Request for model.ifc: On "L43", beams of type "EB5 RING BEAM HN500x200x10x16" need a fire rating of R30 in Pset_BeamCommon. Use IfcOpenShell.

First a look at what the model holds.

```python
import ifcopenshell
import ifcopenshell.util.element

model = ifcopenshell.open("model.ifc")
print(model.schema)
storey = next(s for s in model.by_type("IfcBuildingStorey") if s.Name == "L43")
beams = [e for e in ifcopenshell.util.element.get_decomposition(storey) if e.is_a("IfcBeam")]
seen = {}
for e in beams:
    element_type = ifcopenshell.util.element.get_type(e)
    key = (element_type.Name if element_type != e and element_type else None, ifcopenshell.util.element.get_pset(e, "Pset_BeamCommon", "FireRating"))
    seen[key] = seen.get(key, 0) + 1
for (name, value), count in sorted(seen.items(), key=str):
    print(count, "x", name, "|", value)
```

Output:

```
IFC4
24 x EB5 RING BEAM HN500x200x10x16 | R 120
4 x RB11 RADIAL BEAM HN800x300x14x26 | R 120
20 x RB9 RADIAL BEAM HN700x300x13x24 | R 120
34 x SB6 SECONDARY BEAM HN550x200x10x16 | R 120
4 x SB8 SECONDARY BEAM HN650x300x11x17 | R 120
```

```python
import ifcopenshell
import ifcopenshell.api.pset
import ifcopenshell.util.element

model = ifcopenshell.open("model.ifc")

storey = next(s for s in model.by_type("IfcBuildingStorey") if s.Name == "L43")
beams = [e for e in ifcopenshell.util.element.get_decomposition(storey) if e.is_a("IfcBeam")]

count = 0
for e in beams:
    element_type = ifcopenshell.util.element.get_type(e)
    if element_type in (None, e) or element_type.Name != "EB5 RING BEAM HN500x200x10x16":
        continue
    found = ifcopenshell.util.element.get_pset(e, "Pset_BeamCommon", should_inherit=False)
    if found:
        pset = model.by_id(found["id"])
        if len(ifcopenshell.util.element.get_elements_by_pset(pset)) > 1:
            pset = ifcopenshell.api.pset.unshare_pset(model, products=[e], pset=pset)[0]
    else:
        pset = ifcopenshell.api.pset.add_pset(model, product=e, name="Pset_BeamCommon")
    ifcopenshell.api.pset.edit_pset(model, pset=pset, properties={"FireRating": "R30"})
    count += 1

print(count, "beams updated")

model.write("model-out.ifc")
```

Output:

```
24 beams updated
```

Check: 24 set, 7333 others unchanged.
